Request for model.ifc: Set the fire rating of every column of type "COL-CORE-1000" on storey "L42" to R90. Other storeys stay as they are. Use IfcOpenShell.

First a look at what the model holds.

```python
import ifcopenshell
import ifcopenshell.util.element

model = ifcopenshell.open("model.ifc")
print(model.schema)
storey = next(s for s in model.by_type("IfcBuildingStorey") if s.Name == "L42")
columns = [e for e in ifcopenshell.util.element.get_decomposition(storey) if e.is_a("IfcColumn")]
seen = {}
for e in columns:
    element_type = ifcopenshell.util.element.get_type(e)
    key = (element_type.Name if element_type != e and element_type else None, ifcopenshell.util.element.get_pset(e, "Pset_ColumnCommon", "FireRating"))
    seen[key] = seen.get(key, 0) + 1
for (name, value), count in sorted(seen.items(), key=str):
    print(count, "x", name, "|", value)
```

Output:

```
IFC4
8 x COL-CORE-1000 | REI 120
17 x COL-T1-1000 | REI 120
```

```python
import ifcopenshell
import ifcopenshell.api.pset
import ifcopenshell.util.element

model = ifcopenshell.open("model.ifc")

storey = next(s for s in model.by_type("IfcBuildingStorey") if s.Name == "L42")
columns = [e for e in ifcopenshell.util.element.get_decomposition(storey) if e.is_a("IfcColumn")]

count = 0
for e in columns:
    element_type = ifcopenshell.util.element.get_type(e)
    if element_type in (None, e) or element_type.Name != "COL-CORE-1000":
        continue
    # add_pset returns the element's existing set when there is one.
    pset = ifcopenshell.api.pset.add_pset(model, product=e, name="Pset_ColumnCommon")
    ifcopenshell.api.pset.edit_pset(model, pset=pset, properties={"FireRating": "R90"})
    count += 1

print(count, "columns updated")

model.write("model_edited.ifc")
```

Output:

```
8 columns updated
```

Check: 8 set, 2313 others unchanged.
